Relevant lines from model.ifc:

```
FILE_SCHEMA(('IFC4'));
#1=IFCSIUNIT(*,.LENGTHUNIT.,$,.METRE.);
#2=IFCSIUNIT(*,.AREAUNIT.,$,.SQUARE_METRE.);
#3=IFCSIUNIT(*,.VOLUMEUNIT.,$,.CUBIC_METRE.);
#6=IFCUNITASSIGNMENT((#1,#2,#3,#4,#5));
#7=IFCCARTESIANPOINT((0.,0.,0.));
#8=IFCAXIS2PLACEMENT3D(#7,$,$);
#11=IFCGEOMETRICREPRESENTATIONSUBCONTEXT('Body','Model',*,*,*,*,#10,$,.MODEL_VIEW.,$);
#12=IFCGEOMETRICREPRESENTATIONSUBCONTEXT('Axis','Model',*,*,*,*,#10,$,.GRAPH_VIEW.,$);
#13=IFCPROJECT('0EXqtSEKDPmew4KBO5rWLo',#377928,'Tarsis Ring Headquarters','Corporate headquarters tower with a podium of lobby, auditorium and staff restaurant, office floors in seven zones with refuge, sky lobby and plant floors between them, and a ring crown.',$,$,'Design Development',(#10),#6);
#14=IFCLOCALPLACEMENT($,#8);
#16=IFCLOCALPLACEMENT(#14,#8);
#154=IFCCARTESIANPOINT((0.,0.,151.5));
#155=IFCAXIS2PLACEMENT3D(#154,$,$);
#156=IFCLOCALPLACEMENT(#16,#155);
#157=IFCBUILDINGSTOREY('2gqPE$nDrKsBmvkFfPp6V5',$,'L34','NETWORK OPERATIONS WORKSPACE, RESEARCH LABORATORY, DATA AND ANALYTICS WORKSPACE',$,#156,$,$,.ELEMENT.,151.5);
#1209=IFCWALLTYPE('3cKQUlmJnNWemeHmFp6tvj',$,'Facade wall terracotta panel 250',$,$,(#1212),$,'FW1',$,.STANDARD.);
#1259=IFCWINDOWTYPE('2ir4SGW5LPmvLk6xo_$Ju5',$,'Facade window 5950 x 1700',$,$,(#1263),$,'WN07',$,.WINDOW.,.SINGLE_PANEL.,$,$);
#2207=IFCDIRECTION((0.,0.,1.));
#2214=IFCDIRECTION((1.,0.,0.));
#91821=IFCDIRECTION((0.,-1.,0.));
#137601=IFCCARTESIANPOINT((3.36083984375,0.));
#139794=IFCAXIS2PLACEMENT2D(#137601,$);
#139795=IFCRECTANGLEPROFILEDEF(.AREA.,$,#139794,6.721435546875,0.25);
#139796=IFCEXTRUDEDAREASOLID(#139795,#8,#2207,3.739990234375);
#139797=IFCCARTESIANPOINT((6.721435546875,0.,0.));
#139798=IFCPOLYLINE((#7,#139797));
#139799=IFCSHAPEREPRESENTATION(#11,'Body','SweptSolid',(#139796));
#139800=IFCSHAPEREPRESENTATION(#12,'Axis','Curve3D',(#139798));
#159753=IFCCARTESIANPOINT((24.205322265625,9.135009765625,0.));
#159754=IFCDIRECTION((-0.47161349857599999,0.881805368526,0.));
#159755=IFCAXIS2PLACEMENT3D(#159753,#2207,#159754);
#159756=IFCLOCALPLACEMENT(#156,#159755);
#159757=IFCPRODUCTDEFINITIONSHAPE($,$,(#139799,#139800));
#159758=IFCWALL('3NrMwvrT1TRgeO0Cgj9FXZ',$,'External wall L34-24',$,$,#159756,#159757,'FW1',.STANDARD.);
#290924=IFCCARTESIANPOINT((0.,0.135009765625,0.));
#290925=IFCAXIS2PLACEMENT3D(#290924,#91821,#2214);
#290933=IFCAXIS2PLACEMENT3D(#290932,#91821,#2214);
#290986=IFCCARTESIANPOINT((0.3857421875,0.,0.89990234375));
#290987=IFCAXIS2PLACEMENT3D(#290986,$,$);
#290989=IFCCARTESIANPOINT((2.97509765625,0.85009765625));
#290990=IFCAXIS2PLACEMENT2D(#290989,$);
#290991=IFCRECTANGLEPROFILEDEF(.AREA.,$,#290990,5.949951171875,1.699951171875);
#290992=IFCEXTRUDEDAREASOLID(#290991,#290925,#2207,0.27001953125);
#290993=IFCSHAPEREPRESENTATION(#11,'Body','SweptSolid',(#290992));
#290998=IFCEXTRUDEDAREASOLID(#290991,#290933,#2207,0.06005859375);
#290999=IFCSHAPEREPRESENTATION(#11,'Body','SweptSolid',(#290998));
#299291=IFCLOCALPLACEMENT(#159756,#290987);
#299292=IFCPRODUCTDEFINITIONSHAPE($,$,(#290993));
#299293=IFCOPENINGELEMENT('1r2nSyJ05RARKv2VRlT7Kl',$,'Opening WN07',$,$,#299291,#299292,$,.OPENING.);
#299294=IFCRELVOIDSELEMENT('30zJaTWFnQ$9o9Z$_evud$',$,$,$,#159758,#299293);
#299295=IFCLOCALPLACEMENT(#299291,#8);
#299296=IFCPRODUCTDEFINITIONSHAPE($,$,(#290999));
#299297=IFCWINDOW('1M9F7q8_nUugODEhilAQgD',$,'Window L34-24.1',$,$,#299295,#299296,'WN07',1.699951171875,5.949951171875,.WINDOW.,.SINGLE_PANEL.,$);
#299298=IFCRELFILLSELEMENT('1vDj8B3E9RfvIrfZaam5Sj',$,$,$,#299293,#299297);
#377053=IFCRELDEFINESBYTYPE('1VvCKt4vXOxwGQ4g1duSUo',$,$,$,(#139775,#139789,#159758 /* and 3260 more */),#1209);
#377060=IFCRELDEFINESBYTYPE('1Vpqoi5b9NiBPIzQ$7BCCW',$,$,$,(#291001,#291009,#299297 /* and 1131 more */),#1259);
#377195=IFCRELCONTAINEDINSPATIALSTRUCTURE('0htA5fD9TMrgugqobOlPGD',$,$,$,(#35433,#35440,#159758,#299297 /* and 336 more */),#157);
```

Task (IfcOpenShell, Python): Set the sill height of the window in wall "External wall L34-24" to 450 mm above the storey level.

```python
import numpy as np
import ifcopenshell
import ifcopenshell.api.geometry
import ifcopenshell.geom
import ifcopenshell.util.element
import ifcopenshell.util.placement
import ifcopenshell.util.shape
import ifcopenshell.util.unit

model = ifcopenshell.open("model.ifc")
unit_scale = ifcopenshell.util.unit.calculate_unit_scale(model)

window = model.by_guid("1M9F7q8_nUugODEhilAQgD")
opening = window.FillsVoids[0].RelatingOpeningElement
storey = ifcopenshell.util.element.get_container(window, ifc_class="IfcBuildingStorey")
level = ifcopenshell.util.placement.get_local_placement(storey.ObjectPlacement)[2, 3]

# The opening's origin need not be at the sill, so measure its lowest point.
shape = ifcopenshell.geom.create_shape(ifcopenshell.geom.settings(), opening)
bottom = ifcopenshell.util.shape.get_shape_bottom_elevation(shape, shape.geometry) / unit_scale
dz = level + 0.45 - bottom

shift = np.array([0.0, 0.0, dz])
# The window is placed relative to its opening, so it follows when the opening moves.
matrix = ifcopenshell.util.placement.get_local_placement(opening.ObjectPlacement)
matrix[:3, 3] += shift
ifcopenshell.api.geometry.edit_object_placement(
    model, product=opening, matrix=matrix, is_si=False, should_transform_children=True
)

print(f"moved by {dz * unit_scale:+.3f} m")

model.write("model_v2.ifc")
```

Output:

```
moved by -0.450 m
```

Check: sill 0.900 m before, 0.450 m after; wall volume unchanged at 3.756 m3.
